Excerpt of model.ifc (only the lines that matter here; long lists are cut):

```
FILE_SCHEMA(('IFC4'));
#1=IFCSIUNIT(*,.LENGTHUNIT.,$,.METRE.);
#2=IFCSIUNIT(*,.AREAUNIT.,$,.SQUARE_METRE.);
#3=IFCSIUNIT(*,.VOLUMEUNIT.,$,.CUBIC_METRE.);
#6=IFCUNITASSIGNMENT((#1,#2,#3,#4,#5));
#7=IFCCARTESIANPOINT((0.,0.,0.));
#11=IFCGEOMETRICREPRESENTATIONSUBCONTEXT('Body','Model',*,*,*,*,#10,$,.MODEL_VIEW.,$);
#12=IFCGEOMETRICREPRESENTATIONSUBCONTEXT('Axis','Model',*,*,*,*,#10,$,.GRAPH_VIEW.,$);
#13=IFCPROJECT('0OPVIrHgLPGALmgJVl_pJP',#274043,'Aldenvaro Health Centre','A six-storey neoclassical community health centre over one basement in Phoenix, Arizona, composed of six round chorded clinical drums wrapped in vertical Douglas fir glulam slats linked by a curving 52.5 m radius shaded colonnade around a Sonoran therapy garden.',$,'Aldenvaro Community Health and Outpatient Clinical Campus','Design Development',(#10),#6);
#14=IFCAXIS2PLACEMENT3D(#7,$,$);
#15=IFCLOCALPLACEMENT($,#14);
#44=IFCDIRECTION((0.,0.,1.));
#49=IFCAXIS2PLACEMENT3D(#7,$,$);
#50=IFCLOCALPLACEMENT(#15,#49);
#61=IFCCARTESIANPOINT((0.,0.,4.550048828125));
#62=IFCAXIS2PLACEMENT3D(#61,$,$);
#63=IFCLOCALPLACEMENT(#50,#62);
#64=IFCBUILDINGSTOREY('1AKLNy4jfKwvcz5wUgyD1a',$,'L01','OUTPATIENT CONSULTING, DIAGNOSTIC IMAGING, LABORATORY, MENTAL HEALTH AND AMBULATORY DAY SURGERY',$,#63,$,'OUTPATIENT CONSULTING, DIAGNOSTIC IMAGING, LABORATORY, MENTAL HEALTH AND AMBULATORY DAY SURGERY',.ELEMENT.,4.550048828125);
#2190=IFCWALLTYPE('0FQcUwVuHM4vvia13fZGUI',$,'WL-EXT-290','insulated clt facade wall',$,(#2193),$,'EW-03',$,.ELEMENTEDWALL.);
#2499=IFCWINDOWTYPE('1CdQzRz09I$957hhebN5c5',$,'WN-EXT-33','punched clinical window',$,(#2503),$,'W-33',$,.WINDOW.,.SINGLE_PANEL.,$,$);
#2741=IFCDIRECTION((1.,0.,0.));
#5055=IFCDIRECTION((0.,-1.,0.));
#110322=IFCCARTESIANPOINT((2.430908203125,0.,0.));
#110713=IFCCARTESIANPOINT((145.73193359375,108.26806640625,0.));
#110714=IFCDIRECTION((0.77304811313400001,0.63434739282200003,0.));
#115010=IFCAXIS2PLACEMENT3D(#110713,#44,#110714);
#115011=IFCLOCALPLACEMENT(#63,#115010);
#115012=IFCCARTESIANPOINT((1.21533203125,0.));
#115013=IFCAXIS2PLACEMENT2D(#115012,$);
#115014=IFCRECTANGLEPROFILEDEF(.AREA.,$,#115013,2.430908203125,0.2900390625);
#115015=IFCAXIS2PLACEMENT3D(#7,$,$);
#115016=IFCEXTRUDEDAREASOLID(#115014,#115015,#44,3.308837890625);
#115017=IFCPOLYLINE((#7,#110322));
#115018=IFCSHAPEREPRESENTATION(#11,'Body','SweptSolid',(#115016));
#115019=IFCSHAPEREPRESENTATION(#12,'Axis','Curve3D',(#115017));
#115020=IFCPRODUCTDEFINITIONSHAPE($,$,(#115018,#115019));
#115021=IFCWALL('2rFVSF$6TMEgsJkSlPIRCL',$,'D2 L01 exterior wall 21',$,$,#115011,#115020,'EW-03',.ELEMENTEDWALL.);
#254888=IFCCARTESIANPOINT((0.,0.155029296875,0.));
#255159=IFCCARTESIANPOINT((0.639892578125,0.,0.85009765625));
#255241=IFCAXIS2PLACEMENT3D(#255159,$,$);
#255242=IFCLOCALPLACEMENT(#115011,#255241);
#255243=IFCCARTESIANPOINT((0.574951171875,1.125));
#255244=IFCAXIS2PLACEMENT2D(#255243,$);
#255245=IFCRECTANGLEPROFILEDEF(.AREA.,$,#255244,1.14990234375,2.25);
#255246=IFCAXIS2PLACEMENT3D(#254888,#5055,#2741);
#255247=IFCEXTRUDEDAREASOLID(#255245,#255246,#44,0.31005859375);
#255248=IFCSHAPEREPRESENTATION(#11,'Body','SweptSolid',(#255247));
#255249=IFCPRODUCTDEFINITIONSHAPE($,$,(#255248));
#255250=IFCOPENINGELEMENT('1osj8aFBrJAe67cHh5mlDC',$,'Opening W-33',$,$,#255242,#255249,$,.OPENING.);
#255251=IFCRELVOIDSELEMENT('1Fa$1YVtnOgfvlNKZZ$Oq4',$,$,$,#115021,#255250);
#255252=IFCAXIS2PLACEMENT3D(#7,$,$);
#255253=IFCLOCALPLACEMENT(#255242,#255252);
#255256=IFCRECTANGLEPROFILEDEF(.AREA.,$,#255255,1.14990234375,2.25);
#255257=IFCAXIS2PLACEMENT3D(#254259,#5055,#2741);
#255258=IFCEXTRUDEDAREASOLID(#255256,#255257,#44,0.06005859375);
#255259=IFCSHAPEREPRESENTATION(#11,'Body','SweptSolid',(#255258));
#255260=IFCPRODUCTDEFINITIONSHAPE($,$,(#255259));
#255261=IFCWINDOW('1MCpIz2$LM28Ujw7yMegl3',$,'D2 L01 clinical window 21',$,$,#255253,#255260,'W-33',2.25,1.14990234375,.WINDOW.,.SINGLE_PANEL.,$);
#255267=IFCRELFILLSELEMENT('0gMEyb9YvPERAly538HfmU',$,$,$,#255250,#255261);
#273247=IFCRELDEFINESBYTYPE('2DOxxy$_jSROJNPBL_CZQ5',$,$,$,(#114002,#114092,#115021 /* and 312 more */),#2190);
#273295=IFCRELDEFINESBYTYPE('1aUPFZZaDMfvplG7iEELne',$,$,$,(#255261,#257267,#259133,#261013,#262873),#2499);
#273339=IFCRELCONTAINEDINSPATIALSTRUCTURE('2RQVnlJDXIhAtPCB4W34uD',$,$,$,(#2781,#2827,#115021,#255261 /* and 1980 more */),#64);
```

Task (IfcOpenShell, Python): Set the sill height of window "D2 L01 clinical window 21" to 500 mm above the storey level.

```python
import numpy as np
import ifcopenshell
import ifcopenshell.api.geometry
import ifcopenshell.geom
import ifcopenshell.util.element
import ifcopenshell.util.placement
import ifcopenshell.util.shape
import ifcopenshell.util.unit

model = ifcopenshell.open("model.ifc")
unit_scale = ifcopenshell.util.unit.calculate_unit_scale(model)

window = model.by_id(255261)
opening = window.FillsVoids[0].RelatingOpeningElement
storey = ifcopenshell.util.element.get_container(window, ifc_class="IfcBuildingStorey")
level = ifcopenshell.util.placement.get_local_placement(storey.ObjectPlacement)[2, 3]

# The opening's origin need not be at the sill, so measure its lowest point.
shape = ifcopenshell.geom.create_shape(ifcopenshell.geom.settings(), opening)
bottom = ifcopenshell.util.shape.get_shape_bottom_elevation(shape, shape.geometry) / unit_scale
dz = level + 0.5 / unit_scale - bottom

shift = np.array([0.0, 0.0, dz])
# The window is placed relative to its opening, so it follows when the opening moves.
matrix = ifcopenshell.util.placement.get_local_placement(opening.ObjectPlacement)
matrix[:3, 3] += shift
ifcopenshell.api.geometry.edit_object_placement(
    model, product=opening, matrix=matrix, is_si=False, should_transform_children=True
)

print(f"moved by {dz * unit_scale:+.3f} m")

model.write("model_rev.ifc")
```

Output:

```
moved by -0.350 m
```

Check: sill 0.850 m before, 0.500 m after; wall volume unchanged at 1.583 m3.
